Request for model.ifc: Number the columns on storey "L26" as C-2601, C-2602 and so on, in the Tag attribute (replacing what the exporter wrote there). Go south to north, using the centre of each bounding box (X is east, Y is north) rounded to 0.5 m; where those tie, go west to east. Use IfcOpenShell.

First a look at what the model holds.

```python
import ifcopenshell
import ifcopenshell.util.element
import ifcopenshell.util.placement

model = ifcopenshell.open("model.ifc")
print(model.schema)
storey = next(s for s in model.by_type("IfcBuildingStorey") if s.Name == "L26")
columns = [e for e in ifcopenshell.util.element.get_decomposition(storey) if e.is_a("IfcColumn")]
for e in sorted(columns, key=lambda e: e.id()):
    origin = ifcopenshell.util.placement.get_local_placement(e.ObjectPlacement)[:3, 3]
    print(e.id(), e.Tag, e.Name, origin.round(2) + 0.0, sep=" | ")
```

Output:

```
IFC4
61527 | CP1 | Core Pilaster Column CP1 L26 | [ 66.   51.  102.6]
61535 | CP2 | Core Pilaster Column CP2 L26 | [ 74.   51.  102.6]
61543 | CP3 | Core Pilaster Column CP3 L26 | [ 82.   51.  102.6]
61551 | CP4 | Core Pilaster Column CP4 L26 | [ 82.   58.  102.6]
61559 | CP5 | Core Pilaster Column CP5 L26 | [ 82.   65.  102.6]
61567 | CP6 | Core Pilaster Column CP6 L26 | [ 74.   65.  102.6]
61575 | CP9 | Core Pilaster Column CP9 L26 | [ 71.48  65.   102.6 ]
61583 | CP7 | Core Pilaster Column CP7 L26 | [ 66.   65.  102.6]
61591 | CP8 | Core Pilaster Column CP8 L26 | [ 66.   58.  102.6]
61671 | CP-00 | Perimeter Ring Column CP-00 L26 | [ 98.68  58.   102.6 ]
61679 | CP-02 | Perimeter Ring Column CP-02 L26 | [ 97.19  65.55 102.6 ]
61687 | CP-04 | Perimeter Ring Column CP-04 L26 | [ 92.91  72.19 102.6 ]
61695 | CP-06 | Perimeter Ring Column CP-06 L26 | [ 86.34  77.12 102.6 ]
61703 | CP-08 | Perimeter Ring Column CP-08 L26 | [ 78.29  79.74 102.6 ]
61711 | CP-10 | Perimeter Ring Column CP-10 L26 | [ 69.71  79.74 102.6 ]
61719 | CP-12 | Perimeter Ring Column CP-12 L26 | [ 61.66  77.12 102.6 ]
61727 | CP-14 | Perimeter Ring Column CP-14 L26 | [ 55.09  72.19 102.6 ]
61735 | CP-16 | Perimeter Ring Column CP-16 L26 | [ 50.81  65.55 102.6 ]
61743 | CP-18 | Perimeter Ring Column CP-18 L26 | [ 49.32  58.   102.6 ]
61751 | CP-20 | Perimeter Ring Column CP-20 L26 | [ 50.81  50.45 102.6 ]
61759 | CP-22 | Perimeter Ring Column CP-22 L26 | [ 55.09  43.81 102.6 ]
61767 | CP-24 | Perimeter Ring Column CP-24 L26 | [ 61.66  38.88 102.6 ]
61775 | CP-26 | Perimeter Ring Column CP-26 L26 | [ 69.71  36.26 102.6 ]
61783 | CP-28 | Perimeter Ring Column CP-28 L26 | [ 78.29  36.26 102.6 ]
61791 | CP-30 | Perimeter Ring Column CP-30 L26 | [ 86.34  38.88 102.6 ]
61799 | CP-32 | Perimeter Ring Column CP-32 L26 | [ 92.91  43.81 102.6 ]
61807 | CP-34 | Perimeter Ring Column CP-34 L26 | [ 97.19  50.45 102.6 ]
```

```python
import ifcopenshell
import ifcopenshell.geom
import ifcopenshell.util.element
import ifcopenshell.util.shape

model = ifcopenshell.open("model.ifc")
settings = ifcopenshell.geom.settings()
settings.set("use-world-coords", True)


def centre(element):
    shape = ifcopenshell.geom.create_shape(settings, element)
    return ifcopenshell.util.shape.get_bbox_centroid(shape.geometry)


storey = next(s for s in model.by_type("IfcBuildingStorey") if s.Name == "L26")
columns = [e for e in ifcopenshell.util.element.get_decomposition(storey) if e.is_a("IfcColumn")]

# Insertion points can sit at a corner or the storey origin, so sort by the geometry (in metres).
centres = {e: centre(e) for e in columns}
columns.sort(key=lambda e: (round(centres[e][1] / 0.5), centres[e][0]))

for i, e in enumerate(columns, start=1):
    number = f"C-26{i:02d}"
    e.Tag = number
    print(e.id(), number)

model.write("model_updated.ifc")
```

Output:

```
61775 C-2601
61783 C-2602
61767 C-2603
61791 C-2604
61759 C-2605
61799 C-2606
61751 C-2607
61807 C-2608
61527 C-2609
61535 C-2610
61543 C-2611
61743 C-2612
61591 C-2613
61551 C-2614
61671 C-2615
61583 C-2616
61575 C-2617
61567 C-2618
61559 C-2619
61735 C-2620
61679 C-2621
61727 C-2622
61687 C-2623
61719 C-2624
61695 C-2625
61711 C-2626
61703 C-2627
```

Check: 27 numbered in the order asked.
